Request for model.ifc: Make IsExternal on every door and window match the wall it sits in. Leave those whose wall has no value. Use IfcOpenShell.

First a look at what the model holds.

```python
import ifcopenshell
import ifcopenshell.util.element

model = ifcopenshell.open("model.ifc")
print(model.schema)
seen = {}
for e in model.by_type("IfcDoor") + model.by_type("IfcWindow"):
    if not e.FillsVoids:
        continue
    host = e.FillsVoids[0].RelatingOpeningElement.VoidsElements[0].RelatingBuildingElement
    own = ifcopenshell.util.element.get_pset(e, f"Pset_{e.is_a()[3:].removesuffix('StandardCase')}Common", "IsExternal")
    wall = ifcopenshell.util.element.get_pset(host, "Pset_WallCommon", "IsExternal")
    seen[e.is_a(), own, wall] = seen.get((e.is_a(), own, wall), 0) + 1
for (cls, own, wall), count in sorted(seen.items(), key=str):
    print(count, cls, "IsExternal:", own, "| host wall:", wall)
```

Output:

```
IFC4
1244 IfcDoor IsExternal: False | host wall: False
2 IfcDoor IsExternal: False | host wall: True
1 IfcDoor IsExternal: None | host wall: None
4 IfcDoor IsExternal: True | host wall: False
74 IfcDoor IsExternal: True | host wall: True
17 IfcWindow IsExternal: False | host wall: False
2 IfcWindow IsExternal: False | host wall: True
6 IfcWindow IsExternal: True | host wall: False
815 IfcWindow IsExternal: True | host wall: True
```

```python
import ifcopenshell
import ifcopenshell.api.pset
import ifcopenshell.util.element

model = ifcopenshell.open("model.ifc")

count = 0
for ifc_class, pset_name in (("IfcDoor", "Pset_DoorCommon"), ("IfcWindow", "Pset_WindowCommon")):
    for e in model.by_type(ifc_class):
        if not e.FillsVoids:
            continue
        host = e.FillsVoids[0].RelatingOpeningElement.VoidsElements[0].RelatingBuildingElement
        external = ifcopenshell.util.element.get_pset(host, "Pset_WallCommon", "IsExternal")
        if external is None or ifcopenshell.util.element.get_pset(e, pset_name, "IsExternal") == external:
            continue
        pset = ifcopenshell.api.pset.add_pset(model, product=e, name=pset_name)
        ifcopenshell.api.pset.edit_pset(model, pset=pset, properties={"IsExternal": external})
        count += 1

print(count, "updated")

model.write("model-out.ifc")
```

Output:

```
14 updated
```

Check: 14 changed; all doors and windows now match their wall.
